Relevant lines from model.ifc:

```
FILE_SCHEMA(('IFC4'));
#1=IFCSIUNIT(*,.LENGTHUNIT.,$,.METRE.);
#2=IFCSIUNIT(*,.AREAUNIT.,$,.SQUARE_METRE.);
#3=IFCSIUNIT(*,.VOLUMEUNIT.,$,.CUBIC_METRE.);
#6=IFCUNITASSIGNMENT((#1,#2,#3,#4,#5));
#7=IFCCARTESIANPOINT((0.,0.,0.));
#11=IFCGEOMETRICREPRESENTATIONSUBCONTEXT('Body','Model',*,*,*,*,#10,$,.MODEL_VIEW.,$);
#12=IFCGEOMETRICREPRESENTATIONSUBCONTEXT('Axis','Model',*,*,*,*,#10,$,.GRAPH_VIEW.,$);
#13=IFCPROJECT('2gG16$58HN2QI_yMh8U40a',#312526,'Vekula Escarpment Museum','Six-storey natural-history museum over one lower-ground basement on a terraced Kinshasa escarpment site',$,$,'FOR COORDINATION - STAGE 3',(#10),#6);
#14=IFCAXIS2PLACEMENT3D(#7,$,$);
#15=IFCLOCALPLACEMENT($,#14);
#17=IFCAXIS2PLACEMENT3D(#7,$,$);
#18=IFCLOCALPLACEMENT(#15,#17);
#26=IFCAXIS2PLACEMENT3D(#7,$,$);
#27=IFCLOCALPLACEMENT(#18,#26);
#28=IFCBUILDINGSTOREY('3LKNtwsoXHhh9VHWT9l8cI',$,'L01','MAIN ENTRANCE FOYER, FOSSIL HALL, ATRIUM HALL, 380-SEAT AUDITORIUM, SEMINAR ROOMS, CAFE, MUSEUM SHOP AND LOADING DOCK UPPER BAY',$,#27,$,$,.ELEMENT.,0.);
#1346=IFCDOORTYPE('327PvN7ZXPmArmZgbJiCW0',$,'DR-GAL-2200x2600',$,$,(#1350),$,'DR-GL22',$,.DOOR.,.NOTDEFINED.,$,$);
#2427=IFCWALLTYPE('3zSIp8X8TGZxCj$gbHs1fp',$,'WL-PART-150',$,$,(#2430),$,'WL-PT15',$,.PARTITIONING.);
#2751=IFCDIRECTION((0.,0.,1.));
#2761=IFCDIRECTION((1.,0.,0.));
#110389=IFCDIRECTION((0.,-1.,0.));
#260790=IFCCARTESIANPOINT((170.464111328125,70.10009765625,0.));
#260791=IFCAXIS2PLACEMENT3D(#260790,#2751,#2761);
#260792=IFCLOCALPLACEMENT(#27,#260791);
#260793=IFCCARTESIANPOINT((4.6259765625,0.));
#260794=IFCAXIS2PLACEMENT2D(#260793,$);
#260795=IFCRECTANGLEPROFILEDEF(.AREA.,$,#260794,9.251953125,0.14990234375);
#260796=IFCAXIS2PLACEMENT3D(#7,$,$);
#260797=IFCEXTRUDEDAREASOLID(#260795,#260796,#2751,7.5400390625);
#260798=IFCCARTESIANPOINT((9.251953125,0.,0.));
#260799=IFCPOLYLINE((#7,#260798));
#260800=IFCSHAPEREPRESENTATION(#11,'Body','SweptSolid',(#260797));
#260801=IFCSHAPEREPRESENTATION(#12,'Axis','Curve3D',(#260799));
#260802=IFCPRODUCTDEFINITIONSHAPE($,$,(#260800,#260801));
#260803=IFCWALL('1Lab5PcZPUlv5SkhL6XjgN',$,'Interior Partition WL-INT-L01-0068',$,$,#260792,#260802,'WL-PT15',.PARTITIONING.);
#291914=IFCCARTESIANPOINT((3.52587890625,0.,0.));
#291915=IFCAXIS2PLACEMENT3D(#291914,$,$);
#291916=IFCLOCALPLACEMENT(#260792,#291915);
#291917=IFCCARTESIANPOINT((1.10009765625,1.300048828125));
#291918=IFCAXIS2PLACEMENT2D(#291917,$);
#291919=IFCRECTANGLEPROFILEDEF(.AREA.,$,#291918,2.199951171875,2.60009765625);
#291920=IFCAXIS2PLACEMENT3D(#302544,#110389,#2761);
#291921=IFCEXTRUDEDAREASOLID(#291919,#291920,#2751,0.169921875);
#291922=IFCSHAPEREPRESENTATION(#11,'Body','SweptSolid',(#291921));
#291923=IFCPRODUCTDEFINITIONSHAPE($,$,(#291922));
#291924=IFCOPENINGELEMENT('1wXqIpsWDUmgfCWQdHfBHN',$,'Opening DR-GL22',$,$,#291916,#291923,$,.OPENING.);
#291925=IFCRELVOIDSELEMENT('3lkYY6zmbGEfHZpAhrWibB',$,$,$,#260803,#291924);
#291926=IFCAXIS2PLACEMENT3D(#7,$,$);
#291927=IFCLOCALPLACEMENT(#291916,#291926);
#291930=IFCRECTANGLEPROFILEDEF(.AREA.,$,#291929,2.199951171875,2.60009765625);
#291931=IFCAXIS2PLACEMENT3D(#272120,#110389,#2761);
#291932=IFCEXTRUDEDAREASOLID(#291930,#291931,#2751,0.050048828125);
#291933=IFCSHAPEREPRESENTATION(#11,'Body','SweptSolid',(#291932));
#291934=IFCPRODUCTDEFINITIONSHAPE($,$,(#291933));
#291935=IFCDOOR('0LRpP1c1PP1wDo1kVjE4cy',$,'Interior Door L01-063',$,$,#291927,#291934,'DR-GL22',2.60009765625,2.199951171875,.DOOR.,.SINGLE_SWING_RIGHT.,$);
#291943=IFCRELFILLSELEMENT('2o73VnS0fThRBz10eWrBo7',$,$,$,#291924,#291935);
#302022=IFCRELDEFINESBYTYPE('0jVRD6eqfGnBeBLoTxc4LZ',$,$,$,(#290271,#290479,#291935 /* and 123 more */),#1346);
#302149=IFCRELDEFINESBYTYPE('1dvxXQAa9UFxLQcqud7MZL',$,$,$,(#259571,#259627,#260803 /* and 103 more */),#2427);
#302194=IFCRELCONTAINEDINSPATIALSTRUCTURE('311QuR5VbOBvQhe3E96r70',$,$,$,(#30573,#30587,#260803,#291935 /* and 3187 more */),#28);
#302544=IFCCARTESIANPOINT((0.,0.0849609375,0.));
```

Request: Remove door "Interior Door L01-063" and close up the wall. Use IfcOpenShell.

```python
import ifcopenshell
import ifcopenshell.api.feature
import ifcopenshell.api.root
import ifcopenshell.geom
import ifcopenshell.util.shape

model = ifcopenshell.open("model.ifc")
settings = ifcopenshell.geom.settings()


def volume(element):
    """Net volume in cubic metres, openings subtracted."""
    shape = ifcopenshell.geom.create_shape(settings, element)
    return ifcopenshell.util.shape.get_volume(shape.geometry)


door = model.by_id(291935)
opening = door.FillsVoids[0].RelatingOpeningElement
wall = opening.VoidsElements[0].RelatingBuildingElement
before = volume(wall)

ifcopenshell.api.root.remove_product(model, product=door)
ifcopenshell.api.feature.remove_feature(model, feature=opening)

after = volume(wall)

print(f"wall volume {before:.3f} -> {after:.3f} m3")

model.write("model_edited.ifc")
```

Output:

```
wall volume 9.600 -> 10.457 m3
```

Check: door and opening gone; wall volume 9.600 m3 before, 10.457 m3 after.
